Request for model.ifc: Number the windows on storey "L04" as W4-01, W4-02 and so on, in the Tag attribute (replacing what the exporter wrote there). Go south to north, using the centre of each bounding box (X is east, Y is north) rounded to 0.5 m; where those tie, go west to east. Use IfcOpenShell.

First a look at what the model holds.

```python
import ifcopenshell
import ifcopenshell.util.element
import ifcopenshell.util.placement

model = ifcopenshell.open("model.ifc")
print(model.schema)
storey = next(s for s in model.by_type("IfcBuildingStorey") if s.Name == "L04")
windows = [e for e in ifcopenshell.util.element.get_decomposition(storey) if e.is_a("IfcWindow")]
for e in sorted(windows, key=lambda e: e.id()):
    origin = ifcopenshell.util.placement.get_local_placement(e.ObjectPlacement)[:3, 3]
    print(e.id(), e.Tag, e.Name, origin.round(2) + 0.0, sep=" | ")
```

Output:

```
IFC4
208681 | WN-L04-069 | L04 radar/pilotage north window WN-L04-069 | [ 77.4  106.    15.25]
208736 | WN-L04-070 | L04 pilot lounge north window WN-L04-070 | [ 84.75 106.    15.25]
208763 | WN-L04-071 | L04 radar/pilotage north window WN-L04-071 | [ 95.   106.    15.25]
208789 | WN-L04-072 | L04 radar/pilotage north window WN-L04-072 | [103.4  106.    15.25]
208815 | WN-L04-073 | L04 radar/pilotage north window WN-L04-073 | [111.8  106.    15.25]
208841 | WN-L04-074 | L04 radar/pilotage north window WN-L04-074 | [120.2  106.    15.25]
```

```python
import ifcopenshell
import ifcopenshell.geom
import ifcopenshell.util.element
import ifcopenshell.util.shape

model = ifcopenshell.open("model.ifc")
settings = ifcopenshell.geom.settings()
settings.set("use-world-coords", True)


def centre(element):
    shape = ifcopenshell.geom.create_shape(settings, element)
    return ifcopenshell.util.shape.get_bbox_centroid(shape.geometry)


storey = next(s for s in model.by_type("IfcBuildingStorey") if s.Name == "L04")
windows = [e for e in ifcopenshell.util.element.get_decomposition(storey) if e.is_a("IfcWindow")]

# Insertion points can sit at a corner or the storey origin, so sort by the geometry (in metres).
centres = {e: centre(e) for e in windows}
windows.sort(key=lambda e: (round(centres[e][1] / 0.5), centres[e][0]))

for i, e in enumerate(windows, start=1):
    number = f"W4-{i:02d}"
    e.Tag = number
    print(e.id(), number)

model.write("model-out.ifc")
```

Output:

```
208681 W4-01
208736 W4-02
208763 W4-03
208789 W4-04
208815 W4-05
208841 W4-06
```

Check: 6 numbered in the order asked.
